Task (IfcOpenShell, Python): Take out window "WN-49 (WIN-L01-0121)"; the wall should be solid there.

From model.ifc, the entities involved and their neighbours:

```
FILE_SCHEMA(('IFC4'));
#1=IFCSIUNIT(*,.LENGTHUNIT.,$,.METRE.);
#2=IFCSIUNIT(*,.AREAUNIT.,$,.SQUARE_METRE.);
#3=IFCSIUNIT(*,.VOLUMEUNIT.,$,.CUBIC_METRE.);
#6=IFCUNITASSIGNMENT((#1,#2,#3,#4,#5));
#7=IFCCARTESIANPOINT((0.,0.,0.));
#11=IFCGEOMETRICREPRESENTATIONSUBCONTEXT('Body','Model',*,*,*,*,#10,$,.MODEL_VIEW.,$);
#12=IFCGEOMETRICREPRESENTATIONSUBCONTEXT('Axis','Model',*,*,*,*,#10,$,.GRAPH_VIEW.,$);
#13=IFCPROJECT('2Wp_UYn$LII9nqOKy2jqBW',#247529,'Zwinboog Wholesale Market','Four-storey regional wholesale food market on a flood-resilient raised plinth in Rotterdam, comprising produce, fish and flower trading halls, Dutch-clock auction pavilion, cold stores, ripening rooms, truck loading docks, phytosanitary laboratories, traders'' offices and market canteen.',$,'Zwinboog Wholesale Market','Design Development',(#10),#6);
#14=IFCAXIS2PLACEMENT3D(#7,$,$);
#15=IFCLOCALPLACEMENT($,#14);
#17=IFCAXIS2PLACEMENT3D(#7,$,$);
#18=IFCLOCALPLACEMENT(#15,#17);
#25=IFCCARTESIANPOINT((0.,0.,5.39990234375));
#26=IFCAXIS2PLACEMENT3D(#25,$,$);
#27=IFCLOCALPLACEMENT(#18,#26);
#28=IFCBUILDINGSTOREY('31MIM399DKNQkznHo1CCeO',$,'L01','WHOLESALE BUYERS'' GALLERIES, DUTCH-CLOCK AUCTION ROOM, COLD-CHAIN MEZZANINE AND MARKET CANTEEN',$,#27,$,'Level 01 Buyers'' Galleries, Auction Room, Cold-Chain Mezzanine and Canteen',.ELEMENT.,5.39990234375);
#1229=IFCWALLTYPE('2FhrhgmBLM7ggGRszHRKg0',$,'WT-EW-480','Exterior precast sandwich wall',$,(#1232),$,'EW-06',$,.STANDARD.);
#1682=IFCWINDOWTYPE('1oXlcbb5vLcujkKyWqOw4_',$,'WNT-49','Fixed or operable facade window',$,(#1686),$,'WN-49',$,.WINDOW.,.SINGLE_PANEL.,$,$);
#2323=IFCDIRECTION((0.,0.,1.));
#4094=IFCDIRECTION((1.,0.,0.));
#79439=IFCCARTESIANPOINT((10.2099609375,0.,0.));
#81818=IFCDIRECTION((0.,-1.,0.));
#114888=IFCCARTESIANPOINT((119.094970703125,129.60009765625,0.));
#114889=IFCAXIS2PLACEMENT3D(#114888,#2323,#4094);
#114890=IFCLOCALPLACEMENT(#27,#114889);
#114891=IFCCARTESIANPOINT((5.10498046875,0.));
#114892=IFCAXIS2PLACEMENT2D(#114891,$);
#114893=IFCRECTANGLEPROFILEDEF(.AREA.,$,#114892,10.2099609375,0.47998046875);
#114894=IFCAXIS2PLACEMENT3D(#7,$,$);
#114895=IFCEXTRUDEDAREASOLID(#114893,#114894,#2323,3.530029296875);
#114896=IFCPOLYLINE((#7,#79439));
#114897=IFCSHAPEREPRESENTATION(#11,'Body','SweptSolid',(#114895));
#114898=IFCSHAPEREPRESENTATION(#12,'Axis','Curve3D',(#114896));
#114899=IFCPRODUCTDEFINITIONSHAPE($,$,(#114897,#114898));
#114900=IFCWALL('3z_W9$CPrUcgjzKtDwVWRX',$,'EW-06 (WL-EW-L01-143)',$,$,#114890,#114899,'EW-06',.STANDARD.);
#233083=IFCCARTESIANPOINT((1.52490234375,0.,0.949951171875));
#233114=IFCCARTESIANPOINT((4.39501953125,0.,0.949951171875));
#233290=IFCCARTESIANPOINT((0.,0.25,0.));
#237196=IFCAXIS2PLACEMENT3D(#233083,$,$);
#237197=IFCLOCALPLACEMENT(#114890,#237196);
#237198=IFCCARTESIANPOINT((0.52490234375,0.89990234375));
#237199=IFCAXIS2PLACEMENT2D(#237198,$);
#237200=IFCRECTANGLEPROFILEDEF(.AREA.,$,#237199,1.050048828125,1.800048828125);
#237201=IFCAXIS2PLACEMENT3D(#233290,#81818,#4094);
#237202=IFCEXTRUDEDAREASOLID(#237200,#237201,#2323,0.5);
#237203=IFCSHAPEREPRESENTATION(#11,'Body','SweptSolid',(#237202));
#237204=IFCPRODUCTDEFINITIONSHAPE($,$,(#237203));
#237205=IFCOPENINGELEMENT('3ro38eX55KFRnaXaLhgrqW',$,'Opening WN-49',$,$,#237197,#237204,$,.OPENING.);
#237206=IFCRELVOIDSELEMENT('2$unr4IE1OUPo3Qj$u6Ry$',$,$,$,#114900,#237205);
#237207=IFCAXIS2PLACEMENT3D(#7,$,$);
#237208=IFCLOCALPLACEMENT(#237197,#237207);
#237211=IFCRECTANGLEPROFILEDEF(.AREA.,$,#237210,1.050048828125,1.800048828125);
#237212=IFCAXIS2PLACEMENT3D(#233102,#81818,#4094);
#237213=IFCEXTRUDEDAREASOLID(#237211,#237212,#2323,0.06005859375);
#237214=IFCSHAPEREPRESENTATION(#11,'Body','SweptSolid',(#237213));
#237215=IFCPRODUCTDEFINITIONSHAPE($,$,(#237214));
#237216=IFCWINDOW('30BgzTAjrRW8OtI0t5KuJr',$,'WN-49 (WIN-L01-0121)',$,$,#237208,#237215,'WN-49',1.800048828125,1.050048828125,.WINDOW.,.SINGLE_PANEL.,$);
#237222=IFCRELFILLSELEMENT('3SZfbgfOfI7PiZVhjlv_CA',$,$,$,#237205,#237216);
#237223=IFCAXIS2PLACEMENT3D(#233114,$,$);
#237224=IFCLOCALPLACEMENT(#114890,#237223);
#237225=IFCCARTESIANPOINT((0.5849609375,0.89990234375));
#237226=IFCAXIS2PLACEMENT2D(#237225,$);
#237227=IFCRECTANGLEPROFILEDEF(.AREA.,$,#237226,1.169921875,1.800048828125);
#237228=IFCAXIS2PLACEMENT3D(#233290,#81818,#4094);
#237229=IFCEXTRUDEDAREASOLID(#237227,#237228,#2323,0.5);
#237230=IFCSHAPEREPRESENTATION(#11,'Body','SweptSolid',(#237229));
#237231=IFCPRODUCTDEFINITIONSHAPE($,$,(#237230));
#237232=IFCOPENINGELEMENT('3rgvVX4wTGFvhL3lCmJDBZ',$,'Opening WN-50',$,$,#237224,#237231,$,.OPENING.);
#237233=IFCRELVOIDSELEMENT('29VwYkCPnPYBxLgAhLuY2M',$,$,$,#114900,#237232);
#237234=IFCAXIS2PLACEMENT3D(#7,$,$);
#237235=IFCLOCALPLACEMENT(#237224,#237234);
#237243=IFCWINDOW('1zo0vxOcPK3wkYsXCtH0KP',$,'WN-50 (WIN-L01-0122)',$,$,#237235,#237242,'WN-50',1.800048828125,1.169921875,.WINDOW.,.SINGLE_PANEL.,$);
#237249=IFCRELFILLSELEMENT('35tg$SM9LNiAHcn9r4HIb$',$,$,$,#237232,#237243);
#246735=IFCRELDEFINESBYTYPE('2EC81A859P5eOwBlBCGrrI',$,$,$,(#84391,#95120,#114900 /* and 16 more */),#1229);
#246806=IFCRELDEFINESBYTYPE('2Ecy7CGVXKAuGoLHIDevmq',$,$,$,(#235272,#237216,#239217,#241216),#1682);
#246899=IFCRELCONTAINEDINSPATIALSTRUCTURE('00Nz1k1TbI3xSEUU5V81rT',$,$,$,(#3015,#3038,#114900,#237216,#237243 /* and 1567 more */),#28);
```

```python
import ifcopenshell
import ifcopenshell.api.feature
import ifcopenshell.api.root
import ifcopenshell.geom
import ifcopenshell.util.shape

model = ifcopenshell.open("model.ifc")
settings = ifcopenshell.geom.settings()


def volume(element):
    """Net volume in cubic metres, openings subtracted."""
    shape = ifcopenshell.geom.create_shape(settings, element)
    return ifcopenshell.util.shape.get_volume(shape.geometry)


window = model.by_id(237216)
opening = window.FillsVoids[0].RelatingOpeningElement
wall = opening.VoidsElements[0].RelatingBuildingElement
before = volume(wall)

ifcopenshell.api.root.remove_product(model, product=window)
ifcopenshell.api.feature.remove_feature(model, feature=opening)

after = volume(wall)

print(f"wall volume {before:.3f} -> {after:.3f} m3")

model.write("model-out.ifc")
```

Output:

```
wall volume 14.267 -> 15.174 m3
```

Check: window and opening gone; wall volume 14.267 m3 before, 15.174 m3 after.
